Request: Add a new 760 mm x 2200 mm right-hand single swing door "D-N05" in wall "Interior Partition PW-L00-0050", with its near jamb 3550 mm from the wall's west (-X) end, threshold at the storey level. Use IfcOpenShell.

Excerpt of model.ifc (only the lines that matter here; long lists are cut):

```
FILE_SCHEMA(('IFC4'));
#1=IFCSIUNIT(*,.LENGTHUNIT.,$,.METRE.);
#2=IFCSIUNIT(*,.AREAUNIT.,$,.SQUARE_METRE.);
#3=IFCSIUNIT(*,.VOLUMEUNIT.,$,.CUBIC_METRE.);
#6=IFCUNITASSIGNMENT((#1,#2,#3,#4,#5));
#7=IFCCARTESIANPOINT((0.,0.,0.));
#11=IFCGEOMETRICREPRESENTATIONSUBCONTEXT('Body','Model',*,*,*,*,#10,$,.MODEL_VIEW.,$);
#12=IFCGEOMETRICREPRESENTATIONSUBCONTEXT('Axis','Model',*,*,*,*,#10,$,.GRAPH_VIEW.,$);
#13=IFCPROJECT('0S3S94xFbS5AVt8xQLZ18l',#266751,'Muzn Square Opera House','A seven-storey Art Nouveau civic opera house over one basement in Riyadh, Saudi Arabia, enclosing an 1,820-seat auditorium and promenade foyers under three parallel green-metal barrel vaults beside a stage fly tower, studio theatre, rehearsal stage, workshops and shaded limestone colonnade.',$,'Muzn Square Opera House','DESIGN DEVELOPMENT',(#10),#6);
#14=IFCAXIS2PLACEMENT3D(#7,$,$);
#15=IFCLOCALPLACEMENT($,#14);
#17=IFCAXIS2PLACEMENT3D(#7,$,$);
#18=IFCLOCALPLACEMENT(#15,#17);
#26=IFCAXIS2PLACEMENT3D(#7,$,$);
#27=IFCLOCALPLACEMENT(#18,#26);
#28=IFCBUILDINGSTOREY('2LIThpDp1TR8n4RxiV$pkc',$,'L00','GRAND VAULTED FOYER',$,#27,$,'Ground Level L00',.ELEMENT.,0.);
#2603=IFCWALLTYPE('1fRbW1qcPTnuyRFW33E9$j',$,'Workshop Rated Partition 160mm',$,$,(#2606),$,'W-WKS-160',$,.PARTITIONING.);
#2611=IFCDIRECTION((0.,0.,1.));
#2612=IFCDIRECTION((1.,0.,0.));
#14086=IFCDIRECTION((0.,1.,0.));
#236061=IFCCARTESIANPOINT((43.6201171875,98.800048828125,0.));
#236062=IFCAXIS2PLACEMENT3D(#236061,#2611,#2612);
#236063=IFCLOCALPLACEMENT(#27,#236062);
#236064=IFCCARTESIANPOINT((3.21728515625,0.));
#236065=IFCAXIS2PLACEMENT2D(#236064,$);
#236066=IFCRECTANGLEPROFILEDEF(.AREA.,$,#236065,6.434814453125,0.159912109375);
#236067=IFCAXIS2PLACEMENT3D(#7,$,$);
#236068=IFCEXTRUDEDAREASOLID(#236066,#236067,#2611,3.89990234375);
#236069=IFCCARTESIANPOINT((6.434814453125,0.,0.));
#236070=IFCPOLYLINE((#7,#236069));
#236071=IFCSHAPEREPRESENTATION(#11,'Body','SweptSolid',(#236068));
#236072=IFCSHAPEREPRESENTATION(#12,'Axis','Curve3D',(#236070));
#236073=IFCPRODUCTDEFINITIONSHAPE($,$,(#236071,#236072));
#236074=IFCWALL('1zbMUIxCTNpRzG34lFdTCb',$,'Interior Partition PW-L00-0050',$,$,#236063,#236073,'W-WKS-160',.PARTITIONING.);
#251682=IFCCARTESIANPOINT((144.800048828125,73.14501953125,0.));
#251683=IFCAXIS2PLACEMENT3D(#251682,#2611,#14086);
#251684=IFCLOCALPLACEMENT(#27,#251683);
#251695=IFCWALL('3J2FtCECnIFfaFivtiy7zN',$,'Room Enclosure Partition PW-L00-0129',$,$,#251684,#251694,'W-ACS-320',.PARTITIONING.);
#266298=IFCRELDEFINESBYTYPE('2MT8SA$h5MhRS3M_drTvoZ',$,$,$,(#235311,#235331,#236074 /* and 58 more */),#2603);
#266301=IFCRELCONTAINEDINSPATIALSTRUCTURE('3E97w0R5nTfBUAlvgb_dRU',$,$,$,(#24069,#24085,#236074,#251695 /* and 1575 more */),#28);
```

```python
import numpy as np
import ifcopenshell
import ifcopenshell.api.feature
import ifcopenshell.api.geometry
import ifcopenshell.api.root
import ifcopenshell.api.spatial
import ifcopenshell.geom
import ifcopenshell.util.element
import ifcopenshell.util.placement
import ifcopenshell.util.representation
import ifcopenshell.util.shape
import ifcopenshell.util.unit

model = ifcopenshell.open("model.ifc")
unit_scale = ifcopenshell.util.unit.calculate_unit_scale(model)
settings = ifcopenshell.geom.settings()


def volume(element):
    """Net volume in cubic metres, openings subtracted."""
    shape = ifcopenshell.geom.create_shape(settings, element)
    return ifcopenshell.util.shape.get_volume(shape.geometry)


wall = model.by_guid("1zbMUIxCTNpRzG34lFdTCb")
storey = ifcopenshell.util.element.get_container(wall, ifc_class="IfcBuildingStorey")
context = ifcopenshell.util.representation.get_context(model, "Model", "Body", "MODEL_VIEW")
before = volume(wall)

width, height, from_end, sill = 0.76, 2.2, 3.55, 0.0  # metres

# The wall runs along its own X axis, and the end named is its -X end.
wall_shape = ifcopenshell.geom.create_shape(settings, wall)
x, y, z = ifcopenshell.util.shape.get_vertices(wall_shape.geometry).T
start = x.min() + from_end
face, thickness = float(y.min()), float(y.max() - y.min())
wall_matrix = ifcopenshell.util.placement.get_local_placement(wall.ObjectPlacement)
level = ifcopenshell.util.placement.get_local_placement(storey.ObjectPlacement)[2, 3]


def in_wall(x, y):
    """Placement at x, y metres in the wall's axes, at sill height."""
    matrix = wall_matrix.copy()
    matrix[:, 3] = wall_matrix @ np.array([x / unit_scale, y / unit_scale, 0.0, 1.0])
    matrix[2, 3] = level + sill / unit_scale
    return matrix


# Opening: a box that overshoots both wall faces by 50 mm.
opening = ifcopenshell.api.root.create_entity(model, ifc_class="IfcOpeningElement", predefined_type="OPENING")
box = ifcopenshell.api.geometry.add_wall_representation(
    model, context=context, length=width, height=height, thickness=thickness + 0.1
)
ifcopenshell.api.geometry.assign_representation(model, product=opening, representation=box)
ifcopenshell.api.geometry.edit_object_placement(model, product=opening, matrix=in_wall(start, face - 0.05), is_si=False)
ifcopenshell.api.feature.add_feature(model, feature=opening, element=wall)

door = ifcopenshell.api.root.create_entity(model, ifc_class="IfcDoor", name="D-N05", predefined_type="DOOR")
door.OverallWidth, door.OverallHeight = width / unit_scale, height / unit_scale
door.OperationType = "SINGLE_SWING_RIGHT"
body = ifcopenshell.api.geometry.add_door_representation(
    model,
    context=context,
    overall_width=door.OverallWidth,
    overall_height=door.OverallHeight,
    operation_type="SINGLE_SWING_RIGHT",
    lining_properties={"LiningDepth": thickness / unit_scale, "ThresholdDepth": thickness / unit_scale},
)
ifcopenshell.api.geometry.assign_representation(model, product=door, representation=body)
ifcopenshell.api.spatial.assign_container(model, products=[door], relating_structure=storey)
ifcopenshell.api.feature.add_filling(model, opening=opening, element=door)

# The lining spans the wall, so the door starts at the wall face.
ifcopenshell.api.geometry.edit_object_placement(model, product=door, matrix=in_wall(start, face), is_si=False)

after = volume(wall)

print(f"wall volume {before:.3f} -> {after:.3f} m3")

model.write("model-out.ifc")
```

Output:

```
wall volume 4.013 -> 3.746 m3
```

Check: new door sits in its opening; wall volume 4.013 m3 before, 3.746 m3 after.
